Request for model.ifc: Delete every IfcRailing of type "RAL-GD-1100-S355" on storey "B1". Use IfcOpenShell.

First a look at what the model holds.

```python
import ifcopenshell
import ifcopenshell.util.element

model = ifcopenshell.open("model.ifc")
print(model.schema)
storey = next(s for s in model.by_type("IfcBuildingStorey") if s.Name == "B1")
railings = [e for e in ifcopenshell.util.element.get_decomposition(storey) if e.is_a("IfcRailing")]
seen = {}
for e in railings:
    element_type = ifcopenshell.util.element.get_type(e)
    name = element_type.Name if element_type not in (None, e) else None
    seen[name] = seen.get(name, 0) + 1
for name, count in sorted(seen.items(), key=str):
    print(count, "x", name)
```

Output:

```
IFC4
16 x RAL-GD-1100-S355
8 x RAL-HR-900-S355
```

```python
import ifcopenshell
import ifcopenshell.api.root
import ifcopenshell.util.element

model = ifcopenshell.open("model.ifc")

storey = next(s for s in model.by_type("IfcBuildingStorey") if s.Name == "B1")
railings = [e for e in ifcopenshell.util.element.get_decomposition(storey) if e.is_a("IfcRailing")]
targets = [e for e in railings if (t := ifcopenshell.util.element.get_type(e)) not in (None, e) and t.Name == "RAL-GD-1100-S355"]

for e in targets:
    ifcopenshell.api.root.remove_product(model, product=e)
print(len(targets), "removed")

model.write("model_rev.ifc")
```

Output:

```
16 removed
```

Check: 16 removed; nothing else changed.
